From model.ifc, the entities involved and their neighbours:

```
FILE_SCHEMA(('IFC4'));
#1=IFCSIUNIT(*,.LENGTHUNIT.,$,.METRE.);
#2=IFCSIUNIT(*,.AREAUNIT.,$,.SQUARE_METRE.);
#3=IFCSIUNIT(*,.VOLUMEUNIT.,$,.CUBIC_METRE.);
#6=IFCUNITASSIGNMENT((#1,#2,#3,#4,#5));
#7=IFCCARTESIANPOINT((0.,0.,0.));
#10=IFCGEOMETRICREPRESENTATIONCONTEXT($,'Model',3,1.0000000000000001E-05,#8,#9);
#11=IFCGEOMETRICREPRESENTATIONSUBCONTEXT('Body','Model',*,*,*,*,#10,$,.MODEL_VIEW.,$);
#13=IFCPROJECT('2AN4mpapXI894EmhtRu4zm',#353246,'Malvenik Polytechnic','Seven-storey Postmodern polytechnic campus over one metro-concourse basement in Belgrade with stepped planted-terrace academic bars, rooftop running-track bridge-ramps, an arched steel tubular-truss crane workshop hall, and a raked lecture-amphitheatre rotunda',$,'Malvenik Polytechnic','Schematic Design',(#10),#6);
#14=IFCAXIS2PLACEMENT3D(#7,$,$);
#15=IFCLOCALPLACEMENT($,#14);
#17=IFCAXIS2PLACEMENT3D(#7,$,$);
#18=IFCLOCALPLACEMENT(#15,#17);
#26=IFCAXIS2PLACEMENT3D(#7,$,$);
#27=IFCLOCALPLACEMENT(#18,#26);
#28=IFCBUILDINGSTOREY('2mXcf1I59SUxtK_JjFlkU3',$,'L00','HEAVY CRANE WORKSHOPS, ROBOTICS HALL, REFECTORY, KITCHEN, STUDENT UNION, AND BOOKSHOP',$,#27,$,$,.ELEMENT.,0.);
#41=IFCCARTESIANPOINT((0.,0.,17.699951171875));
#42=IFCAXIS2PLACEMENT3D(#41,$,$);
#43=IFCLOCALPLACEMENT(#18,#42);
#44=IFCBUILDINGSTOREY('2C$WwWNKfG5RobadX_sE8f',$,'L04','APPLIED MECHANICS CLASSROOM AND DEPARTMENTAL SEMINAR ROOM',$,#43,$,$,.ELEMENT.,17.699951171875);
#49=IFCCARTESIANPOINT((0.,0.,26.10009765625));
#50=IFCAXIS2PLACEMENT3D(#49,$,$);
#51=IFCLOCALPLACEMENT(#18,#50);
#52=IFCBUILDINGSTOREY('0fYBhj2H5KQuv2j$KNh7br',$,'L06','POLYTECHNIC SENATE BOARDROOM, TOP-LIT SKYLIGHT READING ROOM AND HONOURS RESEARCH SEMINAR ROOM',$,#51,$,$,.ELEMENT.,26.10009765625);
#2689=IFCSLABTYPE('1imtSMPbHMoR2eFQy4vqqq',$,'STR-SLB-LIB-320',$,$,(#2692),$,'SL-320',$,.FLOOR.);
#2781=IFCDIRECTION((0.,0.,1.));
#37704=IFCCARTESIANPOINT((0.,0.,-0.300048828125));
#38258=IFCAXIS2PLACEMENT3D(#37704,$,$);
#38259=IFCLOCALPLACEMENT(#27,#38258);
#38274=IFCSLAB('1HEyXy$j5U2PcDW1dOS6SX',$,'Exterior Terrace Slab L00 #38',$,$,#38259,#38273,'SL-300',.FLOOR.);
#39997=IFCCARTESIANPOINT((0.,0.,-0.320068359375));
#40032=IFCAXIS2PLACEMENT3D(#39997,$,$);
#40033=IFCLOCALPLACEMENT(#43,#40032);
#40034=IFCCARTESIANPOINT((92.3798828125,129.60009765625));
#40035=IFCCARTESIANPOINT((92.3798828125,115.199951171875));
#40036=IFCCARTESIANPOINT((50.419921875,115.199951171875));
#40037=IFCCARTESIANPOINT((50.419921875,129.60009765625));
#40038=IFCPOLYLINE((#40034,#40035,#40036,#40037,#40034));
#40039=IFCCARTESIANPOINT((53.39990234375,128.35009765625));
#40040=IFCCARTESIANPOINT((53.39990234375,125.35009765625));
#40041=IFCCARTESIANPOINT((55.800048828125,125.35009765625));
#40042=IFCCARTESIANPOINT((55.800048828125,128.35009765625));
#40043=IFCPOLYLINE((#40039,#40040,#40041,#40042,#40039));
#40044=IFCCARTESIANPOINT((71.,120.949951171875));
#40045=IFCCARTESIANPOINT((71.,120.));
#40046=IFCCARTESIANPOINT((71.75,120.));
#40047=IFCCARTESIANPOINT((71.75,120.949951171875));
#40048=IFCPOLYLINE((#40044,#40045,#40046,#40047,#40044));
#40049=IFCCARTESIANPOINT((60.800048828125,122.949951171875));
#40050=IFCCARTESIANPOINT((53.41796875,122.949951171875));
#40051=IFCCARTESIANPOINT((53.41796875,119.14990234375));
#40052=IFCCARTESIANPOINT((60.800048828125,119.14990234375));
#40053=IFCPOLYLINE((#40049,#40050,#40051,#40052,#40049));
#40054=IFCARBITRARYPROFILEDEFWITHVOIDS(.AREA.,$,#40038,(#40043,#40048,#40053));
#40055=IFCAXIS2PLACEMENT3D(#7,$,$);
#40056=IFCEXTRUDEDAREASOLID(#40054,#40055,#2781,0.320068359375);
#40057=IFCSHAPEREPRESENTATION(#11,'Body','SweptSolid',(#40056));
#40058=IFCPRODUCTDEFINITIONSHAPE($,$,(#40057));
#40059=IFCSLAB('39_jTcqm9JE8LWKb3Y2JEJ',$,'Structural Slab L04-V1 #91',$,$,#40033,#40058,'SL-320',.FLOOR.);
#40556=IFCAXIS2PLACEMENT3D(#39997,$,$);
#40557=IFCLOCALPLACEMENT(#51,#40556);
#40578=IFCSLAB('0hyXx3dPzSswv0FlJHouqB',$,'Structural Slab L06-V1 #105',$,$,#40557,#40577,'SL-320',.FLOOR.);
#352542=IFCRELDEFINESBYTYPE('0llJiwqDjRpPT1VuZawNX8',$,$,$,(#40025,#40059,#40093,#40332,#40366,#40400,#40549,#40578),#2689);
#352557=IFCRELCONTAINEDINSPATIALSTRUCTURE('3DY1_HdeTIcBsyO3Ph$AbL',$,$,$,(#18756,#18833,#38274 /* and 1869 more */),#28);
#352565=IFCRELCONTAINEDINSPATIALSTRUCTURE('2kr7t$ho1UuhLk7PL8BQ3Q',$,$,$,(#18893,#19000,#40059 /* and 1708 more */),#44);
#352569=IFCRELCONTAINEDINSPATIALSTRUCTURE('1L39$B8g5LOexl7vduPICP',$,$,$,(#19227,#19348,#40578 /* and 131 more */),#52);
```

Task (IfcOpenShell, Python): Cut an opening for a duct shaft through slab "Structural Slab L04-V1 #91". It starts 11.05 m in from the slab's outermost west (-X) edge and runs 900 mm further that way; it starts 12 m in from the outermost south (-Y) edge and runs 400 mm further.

```python
import numpy as np
import ifcopenshell
import ifcopenshell.api.feature
import ifcopenshell.api.geometry
import ifcopenshell.api.root
import ifcopenshell.geom
import ifcopenshell.util.placement
import ifcopenshell.util.representation
import ifcopenshell.util.shape
import ifcopenshell.util.unit

model = ifcopenshell.open("model.ifc")
unit_scale = ifcopenshell.util.unit.calculate_unit_scale(model)
settings = ifcopenshell.geom.settings()


def volume(element):
    """Net volume in cubic metres, openings subtracted."""
    shape = ifcopenshell.geom.create_shape(settings, element)
    return ifcopenshell.util.shape.get_volume(shape.geometry)


slab = model.by_guid("39_jTcqm9JE8LWKb3Y2JEJ")
before = volume(slab)

# Extent in the slab's own axes, in metres. The edges named are its -X and -Y sides.
slab_shape = ifcopenshell.geom.create_shape(settings, slab)
vertices = ifcopenshell.util.shape.get_vertices(slab_shape.geometry)
x_min, y_min, bottom = vertices.min(axis=0)
top = vertices[:, 2].max()

opening = ifcopenshell.api.root.create_entity(model, ifc_class="IfcOpeningElement", name="Duct shaft opening", predefined_type="OPENING")
context = ifcopenshell.util.representation.get_context(model, "Model", "Body", "MODEL_VIEW")
width, depth = 0.9, 0.4
outline = [(0.0, 0.0), (width, 0.0), (width, depth), (0.0, depth), (0.0, 0.0)]
# Overshoot both faces by 50 mm so the cut is clean.
shape = ifcopenshell.api.geometry.add_slab_representation(
    model, context=context, depth=top - bottom + 0.1, polyline=outline
)
ifcopenshell.api.geometry.assign_representation(model, product=opening, representation=shape)

matrix = ifcopenshell.util.placement.get_local_placement(slab.ObjectPlacement)
matrix[:, 3] = matrix @ np.append(np.array([x_min + 11.05, y_min + 12, bottom - 0.05]) / unit_scale, 1.0)
ifcopenshell.api.geometry.edit_object_placement(model, product=opening, matrix=matrix, is_si=False)
ifcopenshell.api.feature.add_feature(model, feature=opening, element=slab)

after = volume(slab)

print(f"slab volume {before:.3f} -> {after:.3f} m3")

model.write("model_edited.ifc")
```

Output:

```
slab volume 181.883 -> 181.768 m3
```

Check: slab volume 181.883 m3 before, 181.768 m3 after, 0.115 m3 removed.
